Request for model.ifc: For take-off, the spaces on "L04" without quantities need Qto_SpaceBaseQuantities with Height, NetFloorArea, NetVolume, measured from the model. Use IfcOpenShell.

First a look at what the model holds.

```python
import ifcopenshell
import ifcopenshell.util.element
import ifcopenshell.util.unit

model = ifcopenshell.open("model.ifc")
print(model.schema)
for unit_type in ("LENGTHUNIT", "AREAUNIT", "VOLUMEUNIT"):
    print(unit_type, ifcopenshell.util.unit.calculate_unit_scale(model, unit_type))
storey = next(s for s in model.by_type("IfcBuildingStorey") if s.Name == "L04")
spaces = [e for e in ifcopenshell.util.element.get_decomposition(storey) if e.is_a("IfcSpace")]
for e in sorted(spaces, key=lambda e: e.id()):
    print(e.id(), e.is_a(), e.Name, list(ifcopenshell.util.element.get_psets(e, qtos_only=True)), sep=" | ")
```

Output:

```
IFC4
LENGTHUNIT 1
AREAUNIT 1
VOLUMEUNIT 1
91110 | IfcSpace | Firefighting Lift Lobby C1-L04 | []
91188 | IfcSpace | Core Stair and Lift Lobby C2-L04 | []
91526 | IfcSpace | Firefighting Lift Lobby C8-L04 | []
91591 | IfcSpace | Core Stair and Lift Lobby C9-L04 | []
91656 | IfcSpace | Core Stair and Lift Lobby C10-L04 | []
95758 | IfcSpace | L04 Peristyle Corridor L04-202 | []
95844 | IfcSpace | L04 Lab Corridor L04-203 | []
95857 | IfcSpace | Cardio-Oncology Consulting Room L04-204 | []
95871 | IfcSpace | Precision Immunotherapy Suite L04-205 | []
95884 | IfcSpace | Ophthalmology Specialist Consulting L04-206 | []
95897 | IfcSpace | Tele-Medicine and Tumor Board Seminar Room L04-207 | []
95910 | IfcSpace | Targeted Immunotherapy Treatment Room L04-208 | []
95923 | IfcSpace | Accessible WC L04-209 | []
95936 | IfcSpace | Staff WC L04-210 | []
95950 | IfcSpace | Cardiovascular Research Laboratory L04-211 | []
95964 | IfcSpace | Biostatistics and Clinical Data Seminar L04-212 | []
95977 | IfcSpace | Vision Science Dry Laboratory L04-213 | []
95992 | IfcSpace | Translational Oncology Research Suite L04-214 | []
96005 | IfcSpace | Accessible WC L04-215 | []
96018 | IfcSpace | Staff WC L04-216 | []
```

```python
import ifcopenshell
import ifcopenshell.api.pset
import ifcopenshell.geom
import ifcopenshell.util.element
import ifcopenshell.util.shape
import ifcopenshell.util.unit

model = ifcopenshell.open("model.ifc")
unit_scale = ifcopenshell.util.unit.calculate_unit_scale(model)
area_scale = ifcopenshell.util.unit.calculate_unit_scale(model, "AREAUNIT")
volume_scale = ifcopenshell.util.unit.calculate_unit_scale(model, "VOLUMEUNIT")
settings = ifcopenshell.geom.settings()

storey = next(s for s in model.by_type("IfcBuildingStorey") if s.Name == "L04")
spaces = [e for e in ifcopenshell.util.element.get_decomposition(storey) if e.is_a("IfcSpace")]

for e in sorted(spaces, key=lambda e: e.id()):
    if ifcopenshell.util.element.get_psets(e, qtos_only=True, should_inherit=False):
        continue
    # Geometry comes back in metres, in the element's own axes.
    shape = ifcopenshell.geom.create_shape(settings, e)
    values = {
        "Height": ifcopenshell.util.shape.get_z(shape.geometry) / unit_scale,
        "NetFloorArea": ifcopenshell.util.shape.get_footprint_area(shape.geometry) / area_scale,
        "NetVolume": ifcopenshell.util.shape.get_volume(shape.geometry) / volume_scale,
    }
    qto = ifcopenshell.api.pset.add_qto(model, product=e, name="Qto_SpaceBaseQuantities")
    ifcopenshell.api.pset.edit_qto(model, qto=qto, properties=values)
    print(e.id(), {k: round(v, 3) for k, v in values.items()})

model.write("model_rev.ifc")
```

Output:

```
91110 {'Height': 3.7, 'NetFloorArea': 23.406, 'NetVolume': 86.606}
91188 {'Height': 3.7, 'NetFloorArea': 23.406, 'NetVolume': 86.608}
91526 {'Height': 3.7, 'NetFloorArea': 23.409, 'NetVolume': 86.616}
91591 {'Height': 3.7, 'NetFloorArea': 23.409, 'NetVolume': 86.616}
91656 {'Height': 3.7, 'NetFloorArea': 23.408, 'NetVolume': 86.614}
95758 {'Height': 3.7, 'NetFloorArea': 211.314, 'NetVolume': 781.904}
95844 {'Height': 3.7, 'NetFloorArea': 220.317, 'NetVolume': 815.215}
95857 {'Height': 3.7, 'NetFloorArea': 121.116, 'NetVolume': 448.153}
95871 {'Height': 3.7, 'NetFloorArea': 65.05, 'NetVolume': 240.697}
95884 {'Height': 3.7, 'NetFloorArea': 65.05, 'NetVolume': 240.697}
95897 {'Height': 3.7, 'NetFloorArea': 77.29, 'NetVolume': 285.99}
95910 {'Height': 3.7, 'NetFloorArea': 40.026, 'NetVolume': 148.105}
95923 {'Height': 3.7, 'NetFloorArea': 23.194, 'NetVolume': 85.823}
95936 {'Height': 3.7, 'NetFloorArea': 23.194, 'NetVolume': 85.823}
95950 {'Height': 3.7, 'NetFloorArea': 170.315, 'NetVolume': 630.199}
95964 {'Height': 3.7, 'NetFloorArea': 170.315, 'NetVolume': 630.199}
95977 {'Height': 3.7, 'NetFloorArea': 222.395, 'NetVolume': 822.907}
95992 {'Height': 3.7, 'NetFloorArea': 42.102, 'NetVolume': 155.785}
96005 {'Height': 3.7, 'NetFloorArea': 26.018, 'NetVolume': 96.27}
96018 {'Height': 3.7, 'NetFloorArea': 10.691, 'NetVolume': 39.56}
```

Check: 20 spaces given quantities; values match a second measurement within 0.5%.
